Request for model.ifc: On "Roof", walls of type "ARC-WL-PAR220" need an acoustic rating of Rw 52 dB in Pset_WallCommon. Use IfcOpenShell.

First a look at what the model holds.

```python
import ifcopenshell
import ifcopenshell.util.element

model = ifcopenshell.open("model.ifc")
print(model.schema)
storey = next(s for s in model.by_type("IfcBuildingStorey") if s.Name == "Roof")
walls = [e for e in ifcopenshell.util.element.get_decomposition(storey) if e.is_a("IfcWall")]
seen = {}
for e in walls:
    element_type = ifcopenshell.util.element.get_type(e)
    key = (element_type.Name if element_type != e and element_type else None, ifcopenshell.util.element.get_pset(e, "Pset_WallCommon", "AcousticRating"))
    seen[key] = seen.get(key, 0) + 1
for (name, value), count in sorted(seen.items(), key=str):
    print(count, "x", name, "|", value)
```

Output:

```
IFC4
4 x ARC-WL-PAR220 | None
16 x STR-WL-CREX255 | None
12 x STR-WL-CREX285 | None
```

```python
import ifcopenshell
import ifcopenshell.api.pset
import ifcopenshell.util.element

model = ifcopenshell.open("model.ifc")

storey = next(s for s in model.by_type("IfcBuildingStorey") if s.Name == "Roof")
walls = [e for e in ifcopenshell.util.element.get_decomposition(storey) if e.is_a("IfcWall")]

count = 0
for e in walls:
    element_type = ifcopenshell.util.element.get_type(e)
    if element_type in (None, e) or element_type.Name != "ARC-WL-PAR220":
        continue
    # add_pset returns the element's existing set when there is one.
    pset = ifcopenshell.api.pset.add_pset(model, product=e, name="Pset_WallCommon")
    ifcopenshell.api.pset.edit_pset(model, pset=pset, properties={"AcousticRating": "Rw 52 dB"})
    count += 1

print(count, "walls updated")

model.write("model-out.ifc")
```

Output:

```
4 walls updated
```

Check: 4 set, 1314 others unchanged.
